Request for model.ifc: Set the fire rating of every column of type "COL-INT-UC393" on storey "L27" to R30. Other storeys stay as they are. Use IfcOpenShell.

First a look at what the model holds.

```python
import ifcopenshell
import ifcopenshell.util.element

model = ifcopenshell.open("model.ifc")
print(model.schema)
storey = next(s for s in model.by_type("IfcBuildingStorey") if s.Name == "L27")
columns = [e for e in ifcopenshell.util.element.get_decomposition(storey) if e.is_a("IfcColumn")]
seen = {}
for e in columns:
    element_type = ifcopenshell.util.element.get_type(e)
    key = (element_type.Name if element_type != e and element_type else None, ifcopenshell.util.element.get_pset(e, "Pset_ColumnCommon", "FireRating"))
    seen[key] = seen.get(key, 0) + 1
for (name, value), count in sorted(seen.items(), key=str):
    print(count, "x", name, "|", value)
```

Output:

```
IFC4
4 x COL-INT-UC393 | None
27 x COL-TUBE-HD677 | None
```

```python
import ifcopenshell
import ifcopenshell.api.pset
import ifcopenshell.util.element

model = ifcopenshell.open("model.ifc")

storey = next(s for s in model.by_type("IfcBuildingStorey") if s.Name == "L27")
columns = [e for e in ifcopenshell.util.element.get_decomposition(storey) if e.is_a("IfcColumn")]

count = 0
for e in columns:
    element_type = ifcopenshell.util.element.get_type(e)
    if element_type in (None, e) or element_type.Name != "COL-INT-UC393":
        continue
    # add_pset returns the element's existing set when there is one.
    pset = ifcopenshell.api.pset.add_pset(model, product=e, name="Pset_ColumnCommon")
    ifcopenshell.api.pset.edit_pset(model, pset=pset, properties={"FireRating": "R30"})
    count += 1

print(count, "columns updated")

model.write("model-out.ifc")
```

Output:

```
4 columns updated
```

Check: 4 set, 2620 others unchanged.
